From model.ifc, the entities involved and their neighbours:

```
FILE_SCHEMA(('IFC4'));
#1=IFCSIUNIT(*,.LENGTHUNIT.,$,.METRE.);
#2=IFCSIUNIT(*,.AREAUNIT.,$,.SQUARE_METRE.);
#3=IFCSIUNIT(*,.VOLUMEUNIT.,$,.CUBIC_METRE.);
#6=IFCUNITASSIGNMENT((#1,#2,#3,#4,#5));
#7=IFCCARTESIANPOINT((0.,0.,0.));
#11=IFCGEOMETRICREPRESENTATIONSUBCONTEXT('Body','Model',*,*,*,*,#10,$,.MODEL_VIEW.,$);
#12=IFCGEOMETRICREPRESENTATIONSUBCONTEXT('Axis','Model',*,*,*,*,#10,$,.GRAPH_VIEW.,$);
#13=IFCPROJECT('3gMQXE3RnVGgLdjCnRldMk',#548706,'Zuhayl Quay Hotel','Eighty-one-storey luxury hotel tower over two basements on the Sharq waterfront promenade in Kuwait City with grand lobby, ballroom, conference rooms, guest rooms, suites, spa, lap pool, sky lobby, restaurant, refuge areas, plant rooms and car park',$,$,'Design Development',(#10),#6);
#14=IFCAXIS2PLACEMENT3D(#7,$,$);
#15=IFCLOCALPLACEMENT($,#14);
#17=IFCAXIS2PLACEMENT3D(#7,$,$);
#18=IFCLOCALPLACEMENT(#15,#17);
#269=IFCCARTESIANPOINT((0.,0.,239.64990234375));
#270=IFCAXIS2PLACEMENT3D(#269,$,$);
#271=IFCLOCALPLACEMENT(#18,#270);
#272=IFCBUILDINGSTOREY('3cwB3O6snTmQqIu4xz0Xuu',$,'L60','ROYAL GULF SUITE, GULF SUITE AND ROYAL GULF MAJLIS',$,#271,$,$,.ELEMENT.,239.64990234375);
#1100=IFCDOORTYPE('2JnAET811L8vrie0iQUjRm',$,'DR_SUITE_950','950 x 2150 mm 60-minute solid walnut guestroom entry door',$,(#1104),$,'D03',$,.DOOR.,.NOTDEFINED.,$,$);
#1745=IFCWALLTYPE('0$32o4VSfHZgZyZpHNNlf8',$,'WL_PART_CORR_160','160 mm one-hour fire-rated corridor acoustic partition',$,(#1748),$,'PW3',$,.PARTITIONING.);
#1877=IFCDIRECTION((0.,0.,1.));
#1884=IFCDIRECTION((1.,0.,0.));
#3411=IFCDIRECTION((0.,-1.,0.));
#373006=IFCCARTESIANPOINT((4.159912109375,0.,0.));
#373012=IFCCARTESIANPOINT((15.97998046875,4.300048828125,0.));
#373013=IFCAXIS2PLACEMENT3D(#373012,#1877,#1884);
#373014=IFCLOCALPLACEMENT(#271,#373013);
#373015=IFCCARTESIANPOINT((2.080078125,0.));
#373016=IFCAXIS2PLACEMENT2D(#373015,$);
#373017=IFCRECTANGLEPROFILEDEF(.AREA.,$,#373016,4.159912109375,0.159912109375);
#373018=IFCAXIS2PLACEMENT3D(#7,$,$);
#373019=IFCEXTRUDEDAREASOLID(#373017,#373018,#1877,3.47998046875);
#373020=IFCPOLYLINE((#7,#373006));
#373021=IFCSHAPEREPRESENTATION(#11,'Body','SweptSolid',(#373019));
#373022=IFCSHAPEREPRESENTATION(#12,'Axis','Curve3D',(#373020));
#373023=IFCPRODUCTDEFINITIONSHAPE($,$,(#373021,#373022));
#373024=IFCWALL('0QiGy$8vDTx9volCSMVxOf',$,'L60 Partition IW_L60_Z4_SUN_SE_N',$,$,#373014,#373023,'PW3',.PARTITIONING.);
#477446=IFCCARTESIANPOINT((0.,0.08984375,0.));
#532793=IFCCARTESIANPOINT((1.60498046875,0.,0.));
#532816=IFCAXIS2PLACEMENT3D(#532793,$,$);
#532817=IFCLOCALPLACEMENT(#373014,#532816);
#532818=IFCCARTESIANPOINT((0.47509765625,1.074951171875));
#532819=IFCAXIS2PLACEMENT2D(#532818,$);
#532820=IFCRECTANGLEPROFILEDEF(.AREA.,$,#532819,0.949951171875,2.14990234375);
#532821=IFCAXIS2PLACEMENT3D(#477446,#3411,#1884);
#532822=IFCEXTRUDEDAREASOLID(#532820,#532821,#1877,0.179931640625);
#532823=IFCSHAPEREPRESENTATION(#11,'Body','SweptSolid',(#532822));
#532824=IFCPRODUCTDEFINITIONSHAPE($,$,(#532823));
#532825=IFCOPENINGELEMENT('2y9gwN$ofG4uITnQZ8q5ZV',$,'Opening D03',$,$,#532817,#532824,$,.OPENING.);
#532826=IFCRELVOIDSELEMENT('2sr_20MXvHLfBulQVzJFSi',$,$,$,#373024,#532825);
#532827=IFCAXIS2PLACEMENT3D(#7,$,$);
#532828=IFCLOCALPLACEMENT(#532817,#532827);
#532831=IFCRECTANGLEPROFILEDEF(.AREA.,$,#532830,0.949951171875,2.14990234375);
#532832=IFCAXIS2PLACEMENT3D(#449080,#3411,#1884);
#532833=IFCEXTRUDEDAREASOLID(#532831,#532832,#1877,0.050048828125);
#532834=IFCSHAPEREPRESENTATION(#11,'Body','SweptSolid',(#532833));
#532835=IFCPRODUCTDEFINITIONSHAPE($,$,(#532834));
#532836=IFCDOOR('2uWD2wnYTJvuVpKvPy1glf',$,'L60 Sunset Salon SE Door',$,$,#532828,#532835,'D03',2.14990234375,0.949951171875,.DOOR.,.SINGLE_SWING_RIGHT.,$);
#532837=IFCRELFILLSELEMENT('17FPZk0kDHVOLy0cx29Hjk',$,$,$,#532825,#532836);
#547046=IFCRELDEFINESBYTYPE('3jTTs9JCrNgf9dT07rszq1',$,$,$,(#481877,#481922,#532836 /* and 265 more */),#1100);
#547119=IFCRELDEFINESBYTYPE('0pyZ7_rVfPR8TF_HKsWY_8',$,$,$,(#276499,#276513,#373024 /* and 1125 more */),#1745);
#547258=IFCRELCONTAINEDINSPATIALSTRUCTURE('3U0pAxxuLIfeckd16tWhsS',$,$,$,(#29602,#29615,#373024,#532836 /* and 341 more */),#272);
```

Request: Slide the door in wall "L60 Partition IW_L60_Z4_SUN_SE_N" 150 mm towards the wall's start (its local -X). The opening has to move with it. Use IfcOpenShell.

```python
import ifcopenshell
import ifcopenshell.api.geometry
import ifcopenshell.util.placement

model = ifcopenshell.open("model.ifc")

door = model.by_guid("2uWD2wnYTJvuVpKvPy1glf")
opening = door.FillsVoids[0].RelatingOpeningElement
wall = opening.VoidsElements[0].RelatingBuildingElement

wall_matrix = ifcopenshell.util.placement.get_local_placement(wall.ObjectPlacement)
shift = wall_matrix[:3, 0] * -0.15
before = ifcopenshell.util.placement.get_local_placement(door.ObjectPlacement)[:3, 3].copy()

# The door is placed relative to its opening, so it follows when the opening moves.
matrix = ifcopenshell.util.placement.get_local_placement(opening.ObjectPlacement)
matrix[:3, 3] += shift
ifcopenshell.api.geometry.edit_object_placement(
    model, product=opening, matrix=matrix, is_si=False, should_transform_children=True
)

after = ifcopenshell.util.placement.get_local_placement(door.ObjectPlacement)[:3, 3]
print("door moved by", (after - before).round(3) + 0.0)

model.write("model_v2.ifc")
```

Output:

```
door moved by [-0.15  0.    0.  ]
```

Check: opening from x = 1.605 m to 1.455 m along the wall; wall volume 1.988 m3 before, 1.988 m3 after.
